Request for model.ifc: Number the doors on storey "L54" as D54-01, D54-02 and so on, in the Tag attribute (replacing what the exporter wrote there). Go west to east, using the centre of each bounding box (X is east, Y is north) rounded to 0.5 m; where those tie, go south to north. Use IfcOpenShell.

First a look at what the model holds.

```python
import ifcopenshell
import ifcopenshell.util.element
import ifcopenshell.util.placement

model = ifcopenshell.open("model.ifc")
print(model.schema)
storey = next(s for s in model.by_type("IfcBuildingStorey") if s.Name == "L54")
doors = [e for e in ifcopenshell.util.element.get_decomposition(storey) if e.is_a("IfcDoor")]
for e in sorted(doors, key=lambda e: e.id()):
    origin = ifcopenshell.util.placement.get_local_placement(e.ObjectPlacement)[:3, 3]
    print(e.id(), e.Tag, e.Name, origin.round(2) + 0.0, sep=" | ")
```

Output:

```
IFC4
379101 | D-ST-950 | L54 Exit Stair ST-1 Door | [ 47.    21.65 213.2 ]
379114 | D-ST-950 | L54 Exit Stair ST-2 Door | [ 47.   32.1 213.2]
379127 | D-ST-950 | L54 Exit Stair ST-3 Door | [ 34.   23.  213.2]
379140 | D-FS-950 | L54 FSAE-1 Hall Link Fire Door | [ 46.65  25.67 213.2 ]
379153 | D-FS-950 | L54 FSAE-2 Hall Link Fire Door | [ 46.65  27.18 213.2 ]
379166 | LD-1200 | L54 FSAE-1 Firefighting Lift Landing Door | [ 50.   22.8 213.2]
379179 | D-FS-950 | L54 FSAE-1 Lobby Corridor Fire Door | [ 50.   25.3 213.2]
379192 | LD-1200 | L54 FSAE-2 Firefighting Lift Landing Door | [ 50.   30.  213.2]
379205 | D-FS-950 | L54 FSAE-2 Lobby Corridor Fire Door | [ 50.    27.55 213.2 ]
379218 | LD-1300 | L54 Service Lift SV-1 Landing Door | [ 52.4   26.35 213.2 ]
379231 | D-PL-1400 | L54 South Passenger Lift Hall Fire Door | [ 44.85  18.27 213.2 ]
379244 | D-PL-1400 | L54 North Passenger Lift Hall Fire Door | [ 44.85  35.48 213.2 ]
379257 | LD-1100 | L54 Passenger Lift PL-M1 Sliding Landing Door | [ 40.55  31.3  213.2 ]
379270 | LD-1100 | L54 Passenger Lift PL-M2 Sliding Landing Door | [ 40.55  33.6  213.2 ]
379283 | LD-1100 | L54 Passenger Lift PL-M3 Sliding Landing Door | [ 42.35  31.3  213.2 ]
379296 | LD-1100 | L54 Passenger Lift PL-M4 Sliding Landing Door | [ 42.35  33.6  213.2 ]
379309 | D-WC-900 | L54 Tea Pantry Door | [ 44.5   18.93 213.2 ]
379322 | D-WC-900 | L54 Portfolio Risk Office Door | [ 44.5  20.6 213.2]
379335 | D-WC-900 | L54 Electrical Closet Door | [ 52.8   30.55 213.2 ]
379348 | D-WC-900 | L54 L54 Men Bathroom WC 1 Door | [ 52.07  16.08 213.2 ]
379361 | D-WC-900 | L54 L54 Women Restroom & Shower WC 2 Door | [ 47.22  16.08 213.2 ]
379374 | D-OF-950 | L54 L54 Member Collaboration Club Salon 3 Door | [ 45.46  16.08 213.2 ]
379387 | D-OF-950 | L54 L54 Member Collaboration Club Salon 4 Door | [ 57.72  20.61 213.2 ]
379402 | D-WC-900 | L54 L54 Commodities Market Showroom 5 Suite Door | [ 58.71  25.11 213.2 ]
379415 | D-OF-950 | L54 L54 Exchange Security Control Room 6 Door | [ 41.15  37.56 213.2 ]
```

```python
import ifcopenshell
import ifcopenshell.geom
import ifcopenshell.util.element
import ifcopenshell.util.shape

model = ifcopenshell.open("model.ifc")
settings = ifcopenshell.geom.settings()
settings.set("use-world-coords", True)


def centre(element):
    shape = ifcopenshell.geom.create_shape(settings, element)
    return ifcopenshell.util.shape.get_bbox_centroid(shape.geometry)


storey = next(s for s in model.by_type("IfcBuildingStorey") if s.Name == "L54")
doors = [e for e in ifcopenshell.util.element.get_decomposition(storey) if e.is_a("IfcDoor")]

# Insertion points can sit at a corner or the storey origin, so sort by the geometry (in metres).
centres = {e: centre(e) for e in doors}
doors.sort(key=lambda e: (round(centres[e][0] / 0.5), centres[e][1]))

for i, e in enumerate(doors, start=1):
    number = f"D54-{i:02d}"
    e.Tag = number
    print(e.id(), number)

model.write("model-out.ifc")
```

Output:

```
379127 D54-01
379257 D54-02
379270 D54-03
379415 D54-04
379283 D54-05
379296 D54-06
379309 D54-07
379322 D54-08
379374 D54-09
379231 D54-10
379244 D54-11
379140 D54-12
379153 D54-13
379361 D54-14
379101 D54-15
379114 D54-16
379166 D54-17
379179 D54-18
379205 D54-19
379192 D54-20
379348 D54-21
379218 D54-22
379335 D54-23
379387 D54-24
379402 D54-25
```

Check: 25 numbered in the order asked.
